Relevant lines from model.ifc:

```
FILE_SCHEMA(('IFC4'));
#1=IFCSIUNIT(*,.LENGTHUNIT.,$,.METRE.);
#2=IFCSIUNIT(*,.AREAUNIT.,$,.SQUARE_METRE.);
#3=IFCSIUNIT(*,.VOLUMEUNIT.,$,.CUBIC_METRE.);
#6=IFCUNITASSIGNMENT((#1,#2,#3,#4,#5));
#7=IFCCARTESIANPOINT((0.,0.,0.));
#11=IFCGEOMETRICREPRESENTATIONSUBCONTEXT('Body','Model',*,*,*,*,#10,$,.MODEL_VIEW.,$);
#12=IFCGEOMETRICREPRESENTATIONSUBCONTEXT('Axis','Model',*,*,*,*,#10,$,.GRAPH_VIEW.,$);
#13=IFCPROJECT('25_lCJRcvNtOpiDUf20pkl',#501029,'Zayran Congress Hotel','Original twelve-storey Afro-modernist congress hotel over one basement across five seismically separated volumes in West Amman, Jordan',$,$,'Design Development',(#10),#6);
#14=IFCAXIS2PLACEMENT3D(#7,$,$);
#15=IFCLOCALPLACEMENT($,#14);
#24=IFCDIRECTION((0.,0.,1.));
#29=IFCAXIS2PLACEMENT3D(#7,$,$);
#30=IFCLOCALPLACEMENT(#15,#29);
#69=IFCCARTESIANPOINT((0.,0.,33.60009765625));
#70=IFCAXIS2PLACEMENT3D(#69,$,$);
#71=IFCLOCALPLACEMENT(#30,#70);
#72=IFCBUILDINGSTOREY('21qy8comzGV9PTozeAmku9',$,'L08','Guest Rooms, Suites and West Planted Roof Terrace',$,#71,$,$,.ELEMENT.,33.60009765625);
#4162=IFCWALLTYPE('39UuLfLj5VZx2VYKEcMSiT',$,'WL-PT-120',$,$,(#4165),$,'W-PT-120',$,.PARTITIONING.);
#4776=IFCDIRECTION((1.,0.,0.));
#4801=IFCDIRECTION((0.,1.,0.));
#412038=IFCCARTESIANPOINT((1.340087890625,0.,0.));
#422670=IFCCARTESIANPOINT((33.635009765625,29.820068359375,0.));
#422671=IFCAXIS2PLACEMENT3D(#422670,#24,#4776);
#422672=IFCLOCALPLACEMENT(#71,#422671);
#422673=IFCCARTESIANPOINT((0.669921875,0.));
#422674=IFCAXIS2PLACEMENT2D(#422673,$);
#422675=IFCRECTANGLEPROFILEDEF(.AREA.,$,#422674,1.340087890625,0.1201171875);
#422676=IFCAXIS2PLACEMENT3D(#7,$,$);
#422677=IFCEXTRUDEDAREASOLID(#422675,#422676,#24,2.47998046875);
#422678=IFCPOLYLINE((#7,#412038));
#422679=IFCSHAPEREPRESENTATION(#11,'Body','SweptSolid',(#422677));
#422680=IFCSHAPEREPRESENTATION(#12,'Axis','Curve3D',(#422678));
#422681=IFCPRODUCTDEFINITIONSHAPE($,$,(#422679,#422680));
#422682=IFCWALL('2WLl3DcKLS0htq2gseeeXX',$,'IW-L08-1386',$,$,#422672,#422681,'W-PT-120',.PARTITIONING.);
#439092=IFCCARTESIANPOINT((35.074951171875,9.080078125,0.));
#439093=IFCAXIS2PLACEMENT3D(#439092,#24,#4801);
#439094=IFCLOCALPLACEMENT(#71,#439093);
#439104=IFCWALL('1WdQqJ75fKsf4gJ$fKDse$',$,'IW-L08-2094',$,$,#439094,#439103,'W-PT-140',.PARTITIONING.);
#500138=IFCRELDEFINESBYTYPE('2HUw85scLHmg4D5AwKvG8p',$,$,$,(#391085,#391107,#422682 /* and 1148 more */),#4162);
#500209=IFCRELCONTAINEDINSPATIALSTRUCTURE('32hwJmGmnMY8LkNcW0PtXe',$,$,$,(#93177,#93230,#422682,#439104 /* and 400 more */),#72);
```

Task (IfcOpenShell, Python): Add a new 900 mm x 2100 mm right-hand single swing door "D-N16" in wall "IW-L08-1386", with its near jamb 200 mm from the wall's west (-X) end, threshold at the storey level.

```python
import numpy as np
import ifcopenshell
import ifcopenshell.api.feature
import ifcopenshell.api.geometry
import ifcopenshell.api.root
import ifcopenshell.api.spatial
import ifcopenshell.geom
import ifcopenshell.util.element
import ifcopenshell.util.placement
import ifcopenshell.util.representation
import ifcopenshell.util.shape
import ifcopenshell.util.unit

model = ifcopenshell.open("model.ifc")
unit_scale = ifcopenshell.util.unit.calculate_unit_scale(model)
settings = ifcopenshell.geom.settings()


def volume(element):
    """Net volume in cubic metres, openings subtracted."""
    shape = ifcopenshell.geom.create_shape(settings, element)
    return ifcopenshell.util.shape.get_volume(shape.geometry)


wall = model.by_guid("2WLl3DcKLS0htq2gseeeXX")
storey = ifcopenshell.util.element.get_container(wall, ifc_class="IfcBuildingStorey")
context = ifcopenshell.util.representation.get_context(model, "Model", "Body", "MODEL_VIEW")
before = volume(wall)

width, height, from_end, sill = 0.9, 2.1, 0.2, 0.0  # metres

# The wall runs along its own X axis, and the end named is its -X end.
wall_shape = ifcopenshell.geom.create_shape(settings, wall)
x, y, z = ifcopenshell.util.shape.get_vertices(wall_shape.geometry).T
start = x.min() + from_end
face, thickness = float(y.min()), float(y.max() - y.min())
wall_matrix = ifcopenshell.util.placement.get_local_placement(wall.ObjectPlacement)
level = ifcopenshell.util.placement.get_local_placement(storey.ObjectPlacement)[2, 3]


def in_wall(x, y):
    """Placement at x, y metres in the wall's axes, at sill height."""
    matrix = wall_matrix.copy()
    matrix[:, 3] = wall_matrix @ np.array([x / unit_scale, y / unit_scale, 0.0, 1.0])
    matrix[2, 3] = level + sill / unit_scale
    return matrix


# Opening: a box that overshoots both wall faces by 50 mm.
opening = ifcopenshell.api.root.create_entity(model, ifc_class="IfcOpeningElement", predefined_type="OPENING")
box = ifcopenshell.api.geometry.add_wall_representation(
    model, context=context, length=width, height=height, thickness=thickness + 0.1
)
ifcopenshell.api.geometry.assign_representation(model, product=opening, representation=box)
ifcopenshell.api.geometry.edit_object_placement(model, product=opening, matrix=in_wall(start, face - 0.05), is_si=False)
ifcopenshell.api.feature.add_feature(model, feature=opening, element=wall)

door = ifcopenshell.api.root.create_entity(model, ifc_class="IfcDoor", name="D-N16", predefined_type="DOOR")
door.OverallWidth, door.OverallHeight = width / unit_scale, height / unit_scale
door.OperationType = "SINGLE_SWING_RIGHT"
body = ifcopenshell.api.geometry.add_door_representation(
    model,
    context=context,
    overall_width=door.OverallWidth,
    overall_height=door.OverallHeight,
    operation_type="SINGLE_SWING_RIGHT",
    lining_properties={"LiningDepth": thickness / unit_scale, "ThresholdDepth": thickness / unit_scale},
)
ifcopenshell.api.geometry.assign_representation(model, product=door, representation=body)
ifcopenshell.api.spatial.assign_container(model, products=[door], relating_structure=storey)
ifcopenshell.api.feature.add_filling(model, opening=opening, element=door)

# The lining spans the wall, so the door starts at the wall face.
ifcopenshell.api.geometry.edit_object_placement(model, product=door, matrix=in_wall(start, face), is_si=False)

after = volume(wall)

print(f"wall volume {before:.3f} -> {after:.3f} m3")

model.write("model_v2.ifc")
```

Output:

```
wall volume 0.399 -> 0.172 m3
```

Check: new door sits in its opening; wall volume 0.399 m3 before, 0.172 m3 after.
